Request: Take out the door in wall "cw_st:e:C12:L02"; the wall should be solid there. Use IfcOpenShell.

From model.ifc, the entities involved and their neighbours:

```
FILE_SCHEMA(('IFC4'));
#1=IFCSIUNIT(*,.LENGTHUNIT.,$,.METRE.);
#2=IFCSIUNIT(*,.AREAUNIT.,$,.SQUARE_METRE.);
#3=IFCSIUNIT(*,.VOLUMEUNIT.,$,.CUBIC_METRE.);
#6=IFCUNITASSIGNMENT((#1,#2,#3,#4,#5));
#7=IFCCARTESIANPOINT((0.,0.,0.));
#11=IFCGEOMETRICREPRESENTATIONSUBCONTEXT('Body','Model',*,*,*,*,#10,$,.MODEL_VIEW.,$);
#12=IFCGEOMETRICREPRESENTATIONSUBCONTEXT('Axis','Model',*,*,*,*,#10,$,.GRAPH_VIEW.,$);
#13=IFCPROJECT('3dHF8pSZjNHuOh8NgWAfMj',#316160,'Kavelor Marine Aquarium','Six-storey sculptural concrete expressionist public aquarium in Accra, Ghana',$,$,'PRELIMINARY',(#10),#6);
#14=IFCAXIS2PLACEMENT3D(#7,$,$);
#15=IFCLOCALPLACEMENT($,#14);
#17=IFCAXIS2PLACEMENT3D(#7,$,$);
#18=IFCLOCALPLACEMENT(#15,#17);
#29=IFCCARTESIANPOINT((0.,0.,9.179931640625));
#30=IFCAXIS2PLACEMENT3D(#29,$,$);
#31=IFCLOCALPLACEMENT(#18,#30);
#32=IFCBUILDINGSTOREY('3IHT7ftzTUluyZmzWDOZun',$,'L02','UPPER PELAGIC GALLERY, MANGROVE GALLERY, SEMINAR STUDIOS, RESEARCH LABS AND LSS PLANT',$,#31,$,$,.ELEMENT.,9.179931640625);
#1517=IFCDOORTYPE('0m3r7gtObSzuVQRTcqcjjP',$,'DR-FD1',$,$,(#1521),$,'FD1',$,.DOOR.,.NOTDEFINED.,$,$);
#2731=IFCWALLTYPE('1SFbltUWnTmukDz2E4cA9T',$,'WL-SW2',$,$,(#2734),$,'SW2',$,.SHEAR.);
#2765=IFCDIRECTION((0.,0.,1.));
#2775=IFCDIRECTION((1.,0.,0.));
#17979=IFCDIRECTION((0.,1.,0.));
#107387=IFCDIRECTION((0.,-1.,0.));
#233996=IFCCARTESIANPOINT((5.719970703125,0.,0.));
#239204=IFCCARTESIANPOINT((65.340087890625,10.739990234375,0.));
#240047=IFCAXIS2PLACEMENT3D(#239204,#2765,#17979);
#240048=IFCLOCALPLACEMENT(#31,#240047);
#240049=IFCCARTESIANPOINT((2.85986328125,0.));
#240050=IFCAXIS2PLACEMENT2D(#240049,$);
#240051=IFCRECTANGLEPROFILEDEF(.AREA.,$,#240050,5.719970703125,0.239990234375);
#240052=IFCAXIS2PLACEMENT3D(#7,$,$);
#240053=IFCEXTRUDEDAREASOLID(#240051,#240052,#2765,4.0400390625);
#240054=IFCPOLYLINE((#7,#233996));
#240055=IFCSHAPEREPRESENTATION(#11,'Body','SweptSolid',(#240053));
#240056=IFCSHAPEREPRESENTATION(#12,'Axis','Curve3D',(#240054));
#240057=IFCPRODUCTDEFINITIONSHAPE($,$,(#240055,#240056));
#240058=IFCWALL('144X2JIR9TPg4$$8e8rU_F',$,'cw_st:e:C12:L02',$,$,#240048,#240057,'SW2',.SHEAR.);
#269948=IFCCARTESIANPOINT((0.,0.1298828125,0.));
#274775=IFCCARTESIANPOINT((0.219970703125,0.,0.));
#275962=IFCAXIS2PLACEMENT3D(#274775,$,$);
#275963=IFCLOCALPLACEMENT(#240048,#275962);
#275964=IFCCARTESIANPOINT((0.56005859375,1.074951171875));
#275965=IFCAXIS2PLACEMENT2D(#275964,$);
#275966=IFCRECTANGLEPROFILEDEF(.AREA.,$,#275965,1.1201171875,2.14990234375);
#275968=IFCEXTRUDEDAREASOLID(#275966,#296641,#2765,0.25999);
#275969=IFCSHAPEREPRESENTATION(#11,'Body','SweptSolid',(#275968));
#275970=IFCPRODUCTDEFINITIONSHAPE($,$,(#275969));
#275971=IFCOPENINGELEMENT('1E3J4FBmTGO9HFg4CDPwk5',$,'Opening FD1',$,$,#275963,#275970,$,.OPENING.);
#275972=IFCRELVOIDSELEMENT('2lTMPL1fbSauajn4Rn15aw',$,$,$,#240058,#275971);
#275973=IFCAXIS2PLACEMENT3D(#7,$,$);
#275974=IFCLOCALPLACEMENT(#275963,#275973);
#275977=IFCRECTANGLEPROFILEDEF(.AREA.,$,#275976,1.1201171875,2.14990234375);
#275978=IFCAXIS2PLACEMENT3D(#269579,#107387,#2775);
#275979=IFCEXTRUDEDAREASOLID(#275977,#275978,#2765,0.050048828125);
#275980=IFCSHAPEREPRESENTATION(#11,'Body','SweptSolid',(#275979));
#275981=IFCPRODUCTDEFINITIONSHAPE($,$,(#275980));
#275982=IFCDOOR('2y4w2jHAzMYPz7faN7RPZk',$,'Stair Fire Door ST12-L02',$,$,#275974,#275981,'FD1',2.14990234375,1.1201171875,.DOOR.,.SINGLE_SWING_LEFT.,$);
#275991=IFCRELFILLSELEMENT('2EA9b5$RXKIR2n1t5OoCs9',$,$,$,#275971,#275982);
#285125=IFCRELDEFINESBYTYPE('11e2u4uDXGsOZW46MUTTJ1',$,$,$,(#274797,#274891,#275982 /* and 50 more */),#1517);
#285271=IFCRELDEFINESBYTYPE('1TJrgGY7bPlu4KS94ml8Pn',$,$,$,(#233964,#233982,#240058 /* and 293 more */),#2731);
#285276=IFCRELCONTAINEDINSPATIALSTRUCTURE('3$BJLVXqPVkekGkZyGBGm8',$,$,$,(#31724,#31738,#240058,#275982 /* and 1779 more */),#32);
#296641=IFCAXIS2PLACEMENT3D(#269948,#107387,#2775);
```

```python
import ifcopenshell
import ifcopenshell.api.feature
import ifcopenshell.api.root
import ifcopenshell.geom
import ifcopenshell.util.shape

model = ifcopenshell.open("model.ifc")
settings = ifcopenshell.geom.settings()


def volume(element):
    """Net volume in cubic metres, openings subtracted."""
    shape = ifcopenshell.geom.create_shape(settings, element)
    return ifcopenshell.util.shape.get_volume(shape.geometry)


door = model.by_guid("2y4w2jHAzMYPz7faN7RPZk")
opening = door.FillsVoids[0].RelatingOpeningElement
wall = opening.VoidsElements[0].RelatingBuildingElement
before = volume(wall)

ifcopenshell.api.root.remove_product(model, product=door)
ifcopenshell.api.feature.remove_feature(model, feature=opening)

after = volume(wall)

print(f"wall volume {before:.3f} -> {after:.3f} m3")

model.write("model_v2.ifc")
```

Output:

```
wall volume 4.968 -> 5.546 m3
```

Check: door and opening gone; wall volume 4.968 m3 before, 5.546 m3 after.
